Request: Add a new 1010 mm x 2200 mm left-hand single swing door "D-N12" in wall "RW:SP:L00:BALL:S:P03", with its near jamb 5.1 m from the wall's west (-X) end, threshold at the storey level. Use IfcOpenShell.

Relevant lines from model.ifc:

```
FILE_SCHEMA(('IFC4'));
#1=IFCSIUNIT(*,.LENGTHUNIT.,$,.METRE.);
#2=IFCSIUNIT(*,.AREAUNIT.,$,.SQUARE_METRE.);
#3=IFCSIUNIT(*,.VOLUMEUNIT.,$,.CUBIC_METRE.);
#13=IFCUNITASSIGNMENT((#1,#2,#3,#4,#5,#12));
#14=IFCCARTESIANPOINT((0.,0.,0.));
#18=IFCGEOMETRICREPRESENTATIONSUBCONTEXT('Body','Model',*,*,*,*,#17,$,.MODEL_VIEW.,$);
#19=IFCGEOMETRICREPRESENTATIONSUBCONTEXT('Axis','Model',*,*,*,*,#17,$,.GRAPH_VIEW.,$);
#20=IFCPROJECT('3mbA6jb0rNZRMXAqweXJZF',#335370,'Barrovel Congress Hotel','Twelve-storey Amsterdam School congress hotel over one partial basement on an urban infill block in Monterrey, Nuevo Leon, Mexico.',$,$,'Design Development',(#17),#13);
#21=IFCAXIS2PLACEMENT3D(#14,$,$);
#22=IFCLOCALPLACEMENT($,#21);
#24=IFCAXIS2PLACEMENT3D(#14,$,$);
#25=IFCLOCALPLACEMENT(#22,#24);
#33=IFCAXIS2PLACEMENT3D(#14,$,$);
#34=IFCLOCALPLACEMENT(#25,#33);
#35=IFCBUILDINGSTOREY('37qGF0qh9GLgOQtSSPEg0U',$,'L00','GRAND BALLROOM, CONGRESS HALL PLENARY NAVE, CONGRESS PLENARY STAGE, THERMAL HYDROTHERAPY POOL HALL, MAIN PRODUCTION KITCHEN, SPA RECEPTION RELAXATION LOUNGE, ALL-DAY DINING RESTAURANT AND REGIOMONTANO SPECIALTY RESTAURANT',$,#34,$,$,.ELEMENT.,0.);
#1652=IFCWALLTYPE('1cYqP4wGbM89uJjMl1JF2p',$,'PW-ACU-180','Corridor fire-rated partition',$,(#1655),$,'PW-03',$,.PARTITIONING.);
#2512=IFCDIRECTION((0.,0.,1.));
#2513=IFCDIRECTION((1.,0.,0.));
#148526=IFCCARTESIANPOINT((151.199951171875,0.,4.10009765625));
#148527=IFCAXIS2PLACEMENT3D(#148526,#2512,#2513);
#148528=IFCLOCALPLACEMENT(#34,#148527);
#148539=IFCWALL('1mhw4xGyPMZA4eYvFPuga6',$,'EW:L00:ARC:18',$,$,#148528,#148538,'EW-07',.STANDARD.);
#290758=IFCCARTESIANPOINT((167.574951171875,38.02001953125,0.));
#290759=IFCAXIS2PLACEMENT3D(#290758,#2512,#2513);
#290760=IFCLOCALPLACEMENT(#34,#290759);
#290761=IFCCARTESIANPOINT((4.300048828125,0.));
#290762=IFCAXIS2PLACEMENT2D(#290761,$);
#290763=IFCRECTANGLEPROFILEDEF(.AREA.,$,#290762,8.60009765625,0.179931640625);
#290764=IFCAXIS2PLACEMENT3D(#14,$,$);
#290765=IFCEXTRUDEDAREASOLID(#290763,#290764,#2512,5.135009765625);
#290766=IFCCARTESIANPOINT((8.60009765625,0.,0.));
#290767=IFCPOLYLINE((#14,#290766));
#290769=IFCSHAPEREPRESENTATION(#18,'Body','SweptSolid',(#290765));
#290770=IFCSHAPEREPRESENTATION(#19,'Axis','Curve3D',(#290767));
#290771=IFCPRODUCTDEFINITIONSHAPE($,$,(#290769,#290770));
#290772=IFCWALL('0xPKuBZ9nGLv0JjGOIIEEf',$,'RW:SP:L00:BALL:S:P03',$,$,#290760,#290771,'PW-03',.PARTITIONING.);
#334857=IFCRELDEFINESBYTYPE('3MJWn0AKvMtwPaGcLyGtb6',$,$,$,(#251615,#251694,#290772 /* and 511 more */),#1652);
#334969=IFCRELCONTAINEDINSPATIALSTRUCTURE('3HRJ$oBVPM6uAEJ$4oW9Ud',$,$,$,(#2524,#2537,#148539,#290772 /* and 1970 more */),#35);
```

```python
import numpy as np
import ifcopenshell
import ifcopenshell.api.feature
import ifcopenshell.api.geometry
import ifcopenshell.api.root
import ifcopenshell.api.spatial
import ifcopenshell.geom
import ifcopenshell.util.element
import ifcopenshell.util.placement
import ifcopenshell.util.representation
import ifcopenshell.util.shape
import ifcopenshell.util.unit

model = ifcopenshell.open("model.ifc")
unit_scale = ifcopenshell.util.unit.calculate_unit_scale(model)
settings = ifcopenshell.geom.settings()


def volume(element):
    """Net volume in cubic metres, openings subtracted."""
    shape = ifcopenshell.geom.create_shape(settings, element)
    return ifcopenshell.util.shape.get_volume(shape.geometry)


wall = model.by_guid("0xPKuBZ9nGLv0JjGOIIEEf")
storey = ifcopenshell.util.element.get_container(wall, ifc_class="IfcBuildingStorey")
context = ifcopenshell.util.representation.get_context(model, "Model", "Body", "MODEL_VIEW")
before = volume(wall)

width, height, from_end, sill = 1.01, 2.2, 5.1, 0.0  # metres

# The wall runs along its own X axis, and the end named is its -X end.
wall_shape = ifcopenshell.geom.create_shape(settings, wall)
x, y, z = ifcopenshell.util.shape.get_vertices(wall_shape.geometry).T
start = x.min() + from_end
face, thickness = float(y.min()), float(y.max() - y.min())
wall_matrix = ifcopenshell.util.placement.get_local_placement(wall.ObjectPlacement)
level = ifcopenshell.util.placement.get_local_placement(storey.ObjectPlacement)[2, 3]


def in_wall(x, y):
    """Placement at x, y metres in the wall's axes, at sill height."""
    matrix = wall_matrix.copy()
    matrix[:, 3] = wall_matrix @ np.array([x / unit_scale, y / unit_scale, 0.0, 1.0])
    matrix[2, 3] = level + sill / unit_scale
    return matrix


# Opening: a box that overshoots both wall faces by 50 mm.
opening = ifcopenshell.api.root.create_entity(model, ifc_class="IfcOpeningElement", predefined_type="OPENING")
box = ifcopenshell.api.geometry.add_wall_representation(
    model, context=context, length=width, height=height, thickness=thickness + 0.1
)
ifcopenshell.api.geometry.assign_representation(model, product=opening, representation=box)
ifcopenshell.api.geometry.edit_object_placement(model, product=opening, matrix=in_wall(start, face - 0.05), is_si=False)
ifcopenshell.api.feature.add_feature(model, feature=opening, element=wall)

door = ifcopenshell.api.root.create_entity(model, ifc_class="IfcDoor", name="D-N12", predefined_type="DOOR")
door.OverallWidth, door.OverallHeight = width / unit_scale, height / unit_scale
door.OperationType = "SINGLE_SWING_LEFT"
body = ifcopenshell.api.geometry.add_door_representation(
    model,
    context=context,
    overall_width=door.OverallWidth,
    overall_height=door.OverallHeight,
    operation_type="SINGLE_SWING_LEFT",
    lining_properties={"LiningDepth": thickness / unit_scale, "ThresholdDepth": thickness / unit_scale},
)
ifcopenshell.api.geometry.assign_representation(model, product=door, representation=body)
ifcopenshell.api.spatial.assign_container(model, products=[door], relating_structure=storey)
ifcopenshell.api.feature.add_filling(model, opening=opening, element=door)

# The lining spans the wall, so the door starts at the wall face.
ifcopenshell.api.geometry.edit_object_placement(model, product=door, matrix=in_wall(start, face), is_si=False)

after = volume(wall)

print(f"wall volume {before:.3f} -> {after:.3f} m3")

model.write("model_edited.ifc")
```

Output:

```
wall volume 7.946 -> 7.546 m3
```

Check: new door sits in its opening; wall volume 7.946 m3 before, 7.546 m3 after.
